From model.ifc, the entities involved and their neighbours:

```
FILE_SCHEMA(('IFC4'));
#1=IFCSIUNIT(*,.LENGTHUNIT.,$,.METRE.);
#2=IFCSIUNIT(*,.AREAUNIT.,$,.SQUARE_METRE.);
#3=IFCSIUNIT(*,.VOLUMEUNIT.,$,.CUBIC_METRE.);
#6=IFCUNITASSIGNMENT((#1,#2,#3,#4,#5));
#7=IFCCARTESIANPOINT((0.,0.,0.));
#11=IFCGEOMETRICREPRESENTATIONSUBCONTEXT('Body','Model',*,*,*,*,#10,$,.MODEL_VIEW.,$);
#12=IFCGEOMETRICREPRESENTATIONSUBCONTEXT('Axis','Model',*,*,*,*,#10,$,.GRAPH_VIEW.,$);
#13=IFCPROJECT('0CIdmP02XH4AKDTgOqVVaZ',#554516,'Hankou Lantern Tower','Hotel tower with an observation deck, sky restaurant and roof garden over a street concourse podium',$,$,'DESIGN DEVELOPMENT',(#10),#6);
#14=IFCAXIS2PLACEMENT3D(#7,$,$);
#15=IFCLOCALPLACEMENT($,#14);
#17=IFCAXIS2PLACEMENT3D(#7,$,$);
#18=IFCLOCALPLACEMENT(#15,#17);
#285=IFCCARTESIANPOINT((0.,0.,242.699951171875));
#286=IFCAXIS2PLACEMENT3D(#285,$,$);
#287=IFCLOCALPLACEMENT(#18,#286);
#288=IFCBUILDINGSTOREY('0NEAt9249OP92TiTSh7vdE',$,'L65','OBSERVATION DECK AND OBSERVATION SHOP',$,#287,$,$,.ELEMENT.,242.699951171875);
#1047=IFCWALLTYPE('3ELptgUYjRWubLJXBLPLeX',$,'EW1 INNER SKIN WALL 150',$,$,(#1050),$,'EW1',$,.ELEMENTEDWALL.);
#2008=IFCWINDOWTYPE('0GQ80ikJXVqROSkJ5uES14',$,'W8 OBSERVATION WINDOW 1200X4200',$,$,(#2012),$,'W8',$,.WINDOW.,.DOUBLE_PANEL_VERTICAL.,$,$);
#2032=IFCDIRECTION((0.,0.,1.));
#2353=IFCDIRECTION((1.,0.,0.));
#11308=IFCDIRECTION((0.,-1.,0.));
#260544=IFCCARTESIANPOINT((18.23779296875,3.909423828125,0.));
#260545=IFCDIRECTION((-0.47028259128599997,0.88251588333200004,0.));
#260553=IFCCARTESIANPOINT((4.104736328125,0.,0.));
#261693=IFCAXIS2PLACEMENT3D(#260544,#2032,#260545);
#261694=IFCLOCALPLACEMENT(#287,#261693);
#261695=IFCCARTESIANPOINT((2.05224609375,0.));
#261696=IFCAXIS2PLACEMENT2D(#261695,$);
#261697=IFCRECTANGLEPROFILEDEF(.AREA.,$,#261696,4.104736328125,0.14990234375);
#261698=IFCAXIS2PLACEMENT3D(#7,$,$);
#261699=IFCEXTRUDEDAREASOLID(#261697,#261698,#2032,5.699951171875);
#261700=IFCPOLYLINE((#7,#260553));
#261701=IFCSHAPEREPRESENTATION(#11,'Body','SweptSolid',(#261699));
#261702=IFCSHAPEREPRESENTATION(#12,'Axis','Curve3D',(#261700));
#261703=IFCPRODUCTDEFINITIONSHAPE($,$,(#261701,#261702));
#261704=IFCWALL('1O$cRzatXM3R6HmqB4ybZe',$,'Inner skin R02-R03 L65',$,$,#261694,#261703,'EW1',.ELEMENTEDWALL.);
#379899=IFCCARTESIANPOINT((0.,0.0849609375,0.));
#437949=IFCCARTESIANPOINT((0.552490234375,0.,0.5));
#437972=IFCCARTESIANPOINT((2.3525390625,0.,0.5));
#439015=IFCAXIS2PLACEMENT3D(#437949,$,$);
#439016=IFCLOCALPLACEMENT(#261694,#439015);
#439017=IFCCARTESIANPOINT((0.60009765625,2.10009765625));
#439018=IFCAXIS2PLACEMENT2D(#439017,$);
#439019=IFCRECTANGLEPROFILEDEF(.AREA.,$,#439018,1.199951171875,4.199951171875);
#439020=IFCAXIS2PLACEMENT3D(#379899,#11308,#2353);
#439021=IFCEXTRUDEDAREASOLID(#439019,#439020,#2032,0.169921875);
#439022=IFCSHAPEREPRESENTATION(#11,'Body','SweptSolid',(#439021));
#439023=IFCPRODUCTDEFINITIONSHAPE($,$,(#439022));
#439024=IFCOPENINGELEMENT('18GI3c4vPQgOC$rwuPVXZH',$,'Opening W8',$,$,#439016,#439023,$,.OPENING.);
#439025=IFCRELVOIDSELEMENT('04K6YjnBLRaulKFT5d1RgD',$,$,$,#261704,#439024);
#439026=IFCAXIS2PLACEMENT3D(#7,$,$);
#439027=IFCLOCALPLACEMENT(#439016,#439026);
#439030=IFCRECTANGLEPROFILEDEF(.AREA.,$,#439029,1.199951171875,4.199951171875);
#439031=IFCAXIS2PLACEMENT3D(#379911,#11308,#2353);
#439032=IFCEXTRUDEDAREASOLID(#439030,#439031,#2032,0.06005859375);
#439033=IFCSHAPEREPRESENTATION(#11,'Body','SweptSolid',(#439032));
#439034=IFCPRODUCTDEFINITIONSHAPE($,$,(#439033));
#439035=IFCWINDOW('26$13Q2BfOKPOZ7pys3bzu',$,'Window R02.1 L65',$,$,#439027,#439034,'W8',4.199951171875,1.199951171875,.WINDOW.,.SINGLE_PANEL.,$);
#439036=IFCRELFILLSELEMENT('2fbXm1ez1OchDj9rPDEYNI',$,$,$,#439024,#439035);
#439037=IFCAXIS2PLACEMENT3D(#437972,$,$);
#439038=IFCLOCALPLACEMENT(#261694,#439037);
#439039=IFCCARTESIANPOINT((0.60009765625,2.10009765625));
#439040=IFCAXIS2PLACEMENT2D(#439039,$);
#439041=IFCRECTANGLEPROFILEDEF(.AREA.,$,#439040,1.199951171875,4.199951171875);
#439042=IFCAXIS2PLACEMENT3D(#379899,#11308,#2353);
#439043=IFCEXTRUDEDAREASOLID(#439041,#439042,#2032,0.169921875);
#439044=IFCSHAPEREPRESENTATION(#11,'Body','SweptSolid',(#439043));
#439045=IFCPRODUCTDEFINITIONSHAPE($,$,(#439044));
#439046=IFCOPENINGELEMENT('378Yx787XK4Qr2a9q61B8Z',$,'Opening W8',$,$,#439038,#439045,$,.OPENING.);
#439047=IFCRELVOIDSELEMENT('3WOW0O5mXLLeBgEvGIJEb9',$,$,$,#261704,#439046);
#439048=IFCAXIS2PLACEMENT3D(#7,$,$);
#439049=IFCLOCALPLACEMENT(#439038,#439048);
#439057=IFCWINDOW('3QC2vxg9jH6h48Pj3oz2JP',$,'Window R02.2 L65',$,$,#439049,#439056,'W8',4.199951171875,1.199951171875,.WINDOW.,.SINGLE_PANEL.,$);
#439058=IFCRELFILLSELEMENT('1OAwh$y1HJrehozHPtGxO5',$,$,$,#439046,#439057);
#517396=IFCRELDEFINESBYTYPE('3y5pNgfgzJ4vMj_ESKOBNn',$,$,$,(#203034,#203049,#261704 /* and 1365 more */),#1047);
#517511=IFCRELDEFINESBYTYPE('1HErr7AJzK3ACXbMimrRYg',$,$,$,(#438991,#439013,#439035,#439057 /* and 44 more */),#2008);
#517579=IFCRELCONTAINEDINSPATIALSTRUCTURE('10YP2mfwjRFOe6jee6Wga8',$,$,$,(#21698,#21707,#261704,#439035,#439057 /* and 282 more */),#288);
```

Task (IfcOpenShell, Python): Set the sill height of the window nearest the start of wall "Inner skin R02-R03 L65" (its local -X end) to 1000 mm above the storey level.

```python
import numpy as np
import ifcopenshell
import ifcopenshell.api.geometry
import ifcopenshell.geom
import ifcopenshell.util.element
import ifcopenshell.util.placement
import ifcopenshell.util.shape
import ifcopenshell.util.unit

model = ifcopenshell.open("model.ifc")
unit_scale = ifcopenshell.util.unit.calculate_unit_scale(model)

window = model.by_guid("26$13Q2BfOKPOZ7pys3bzu")
opening = window.FillsVoids[0].RelatingOpeningElement
storey = ifcopenshell.util.element.get_container(window, ifc_class="IfcBuildingStorey")
level = ifcopenshell.util.placement.get_local_placement(storey.ObjectPlacement)[2, 3]

# The opening's origin need not be at the sill, so measure its lowest point.
shape = ifcopenshell.geom.create_shape(ifcopenshell.geom.settings(), opening)
bottom = ifcopenshell.util.shape.get_shape_bottom_elevation(shape, shape.geometry) / unit_scale
dz = level + 1 / unit_scale - bottom

shift = np.array([0.0, 0.0, dz])
# The window is placed relative to its opening, so it follows when the opening moves.
matrix = ifcopenshell.util.placement.get_local_placement(opening.ObjectPlacement)
matrix[:3, 3] += shift
ifcopenshell.api.geometry.edit_object_placement(
    model, product=opening, matrix=matrix, is_si=False, should_transform_children=True
)

print(f"moved by {dz * unit_scale:+.3f} m")

model.write("model_edited.ifc")
```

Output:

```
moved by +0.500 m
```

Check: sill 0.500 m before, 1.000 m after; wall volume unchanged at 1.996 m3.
